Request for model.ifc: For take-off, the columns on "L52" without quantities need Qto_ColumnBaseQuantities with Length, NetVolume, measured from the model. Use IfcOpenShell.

First a look at what the model holds.

```python
import ifcopenshell
import ifcopenshell.util.element
import ifcopenshell.util.unit

model = ifcopenshell.open("model.ifc")
print(model.schema)
for unit_type in ("LENGTHUNIT", "AREAUNIT", "VOLUMEUNIT"):
    print(unit_type, ifcopenshell.util.unit.calculate_unit_scale(model, unit_type))
storey = next(s for s in model.by_type("IfcBuildingStorey") if s.Name == "L52")
columns = [e for e in ifcopenshell.util.element.get_decomposition(storey) if e.is_a("IfcColumn")]
for e in sorted(columns, key=lambda e: e.id()):
    print(e.id(), e.is_a(), e.Name, list(ifcopenshell.util.element.get_psets(e, qtos_only=True)), sep=" | ")
```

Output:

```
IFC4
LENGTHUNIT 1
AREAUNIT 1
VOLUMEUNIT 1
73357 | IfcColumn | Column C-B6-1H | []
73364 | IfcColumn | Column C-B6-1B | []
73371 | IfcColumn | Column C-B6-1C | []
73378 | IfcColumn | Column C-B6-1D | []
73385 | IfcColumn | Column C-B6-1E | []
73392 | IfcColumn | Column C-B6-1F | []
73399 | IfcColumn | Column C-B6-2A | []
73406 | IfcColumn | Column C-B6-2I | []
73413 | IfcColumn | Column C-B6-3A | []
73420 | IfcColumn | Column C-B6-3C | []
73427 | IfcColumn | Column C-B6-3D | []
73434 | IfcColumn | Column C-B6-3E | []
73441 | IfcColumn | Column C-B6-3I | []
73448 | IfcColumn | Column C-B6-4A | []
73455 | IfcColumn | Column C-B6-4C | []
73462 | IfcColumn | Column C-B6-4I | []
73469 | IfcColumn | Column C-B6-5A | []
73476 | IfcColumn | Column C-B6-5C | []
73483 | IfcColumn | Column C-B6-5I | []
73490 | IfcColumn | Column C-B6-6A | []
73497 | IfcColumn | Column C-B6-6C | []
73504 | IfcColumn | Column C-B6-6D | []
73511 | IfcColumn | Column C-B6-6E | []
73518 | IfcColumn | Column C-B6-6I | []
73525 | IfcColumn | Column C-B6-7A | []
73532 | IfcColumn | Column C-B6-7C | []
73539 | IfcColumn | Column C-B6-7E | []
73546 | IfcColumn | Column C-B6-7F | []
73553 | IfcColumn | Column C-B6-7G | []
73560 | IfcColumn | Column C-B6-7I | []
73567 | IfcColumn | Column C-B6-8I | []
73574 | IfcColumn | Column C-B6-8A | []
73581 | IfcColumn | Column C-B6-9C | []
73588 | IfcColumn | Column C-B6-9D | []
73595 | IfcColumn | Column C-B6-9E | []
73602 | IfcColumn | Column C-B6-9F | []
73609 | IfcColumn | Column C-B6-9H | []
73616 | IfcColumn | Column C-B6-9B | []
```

```python
import ifcopenshell
import ifcopenshell.api.pset
import ifcopenshell.geom
import ifcopenshell.util.element
import ifcopenshell.util.shape
import ifcopenshell.util.unit

model = ifcopenshell.open("model.ifc")
unit_scale = ifcopenshell.util.unit.calculate_unit_scale(model)
volume_scale = ifcopenshell.util.unit.calculate_unit_scale(model, "VOLUMEUNIT")
settings = ifcopenshell.geom.settings()

storey = next(s for s in model.by_type("IfcBuildingStorey") if s.Name == "L52")
columns = [e for e in ifcopenshell.util.element.get_decomposition(storey) if e.is_a("IfcColumn")]

for e in sorted(columns, key=lambda e: e.id()):
    if ifcopenshell.util.element.get_psets(e, qtos_only=True, should_inherit=False):
        continue
    # Geometry comes back in metres, in the element's own axes.
    shape = ifcopenshell.geom.create_shape(settings, e)
    values = {
        "Length": ifcopenshell.util.shape.get_z(shape.geometry) / unit_scale,
        "NetVolume": ifcopenshell.util.shape.get_volume(shape.geometry) / volume_scale,
    }
    qto = ifcopenshell.api.pset.add_qto(model, product=e, name="Qto_ColumnBaseQuantities")
    ifcopenshell.api.pset.edit_qto(model, qto=qto, properties=values)
    print(e.id(), {k: round(v, 3) for k, v in values.items()})

model.write("model_v2.ifc")
```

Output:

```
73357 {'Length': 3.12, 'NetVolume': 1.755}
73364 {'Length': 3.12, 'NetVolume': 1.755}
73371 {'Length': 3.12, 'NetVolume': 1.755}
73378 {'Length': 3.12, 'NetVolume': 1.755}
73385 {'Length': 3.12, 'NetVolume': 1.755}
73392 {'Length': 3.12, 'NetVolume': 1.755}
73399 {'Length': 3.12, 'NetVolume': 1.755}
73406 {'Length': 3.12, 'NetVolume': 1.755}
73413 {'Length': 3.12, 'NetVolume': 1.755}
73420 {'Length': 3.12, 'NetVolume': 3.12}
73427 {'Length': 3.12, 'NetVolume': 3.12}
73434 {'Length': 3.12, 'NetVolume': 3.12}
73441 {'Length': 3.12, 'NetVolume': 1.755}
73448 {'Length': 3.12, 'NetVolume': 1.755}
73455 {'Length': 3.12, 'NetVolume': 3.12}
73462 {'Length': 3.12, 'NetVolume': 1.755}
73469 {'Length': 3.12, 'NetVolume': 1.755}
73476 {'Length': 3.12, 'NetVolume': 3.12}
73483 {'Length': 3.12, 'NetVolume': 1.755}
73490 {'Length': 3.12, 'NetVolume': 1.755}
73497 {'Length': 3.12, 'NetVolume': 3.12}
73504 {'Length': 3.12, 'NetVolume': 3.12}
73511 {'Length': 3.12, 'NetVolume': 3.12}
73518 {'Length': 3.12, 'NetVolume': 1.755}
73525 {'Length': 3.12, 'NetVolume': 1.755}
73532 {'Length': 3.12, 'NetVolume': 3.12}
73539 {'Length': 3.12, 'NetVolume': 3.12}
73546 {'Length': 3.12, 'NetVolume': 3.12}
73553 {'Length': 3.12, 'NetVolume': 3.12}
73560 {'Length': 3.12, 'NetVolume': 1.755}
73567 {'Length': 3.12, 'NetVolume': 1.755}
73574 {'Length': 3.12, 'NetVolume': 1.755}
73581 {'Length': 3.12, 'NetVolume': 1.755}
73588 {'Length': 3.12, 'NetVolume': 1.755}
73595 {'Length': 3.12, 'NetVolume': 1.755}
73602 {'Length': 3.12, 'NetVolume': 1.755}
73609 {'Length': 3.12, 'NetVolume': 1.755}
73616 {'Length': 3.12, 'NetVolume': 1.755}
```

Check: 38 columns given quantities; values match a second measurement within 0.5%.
